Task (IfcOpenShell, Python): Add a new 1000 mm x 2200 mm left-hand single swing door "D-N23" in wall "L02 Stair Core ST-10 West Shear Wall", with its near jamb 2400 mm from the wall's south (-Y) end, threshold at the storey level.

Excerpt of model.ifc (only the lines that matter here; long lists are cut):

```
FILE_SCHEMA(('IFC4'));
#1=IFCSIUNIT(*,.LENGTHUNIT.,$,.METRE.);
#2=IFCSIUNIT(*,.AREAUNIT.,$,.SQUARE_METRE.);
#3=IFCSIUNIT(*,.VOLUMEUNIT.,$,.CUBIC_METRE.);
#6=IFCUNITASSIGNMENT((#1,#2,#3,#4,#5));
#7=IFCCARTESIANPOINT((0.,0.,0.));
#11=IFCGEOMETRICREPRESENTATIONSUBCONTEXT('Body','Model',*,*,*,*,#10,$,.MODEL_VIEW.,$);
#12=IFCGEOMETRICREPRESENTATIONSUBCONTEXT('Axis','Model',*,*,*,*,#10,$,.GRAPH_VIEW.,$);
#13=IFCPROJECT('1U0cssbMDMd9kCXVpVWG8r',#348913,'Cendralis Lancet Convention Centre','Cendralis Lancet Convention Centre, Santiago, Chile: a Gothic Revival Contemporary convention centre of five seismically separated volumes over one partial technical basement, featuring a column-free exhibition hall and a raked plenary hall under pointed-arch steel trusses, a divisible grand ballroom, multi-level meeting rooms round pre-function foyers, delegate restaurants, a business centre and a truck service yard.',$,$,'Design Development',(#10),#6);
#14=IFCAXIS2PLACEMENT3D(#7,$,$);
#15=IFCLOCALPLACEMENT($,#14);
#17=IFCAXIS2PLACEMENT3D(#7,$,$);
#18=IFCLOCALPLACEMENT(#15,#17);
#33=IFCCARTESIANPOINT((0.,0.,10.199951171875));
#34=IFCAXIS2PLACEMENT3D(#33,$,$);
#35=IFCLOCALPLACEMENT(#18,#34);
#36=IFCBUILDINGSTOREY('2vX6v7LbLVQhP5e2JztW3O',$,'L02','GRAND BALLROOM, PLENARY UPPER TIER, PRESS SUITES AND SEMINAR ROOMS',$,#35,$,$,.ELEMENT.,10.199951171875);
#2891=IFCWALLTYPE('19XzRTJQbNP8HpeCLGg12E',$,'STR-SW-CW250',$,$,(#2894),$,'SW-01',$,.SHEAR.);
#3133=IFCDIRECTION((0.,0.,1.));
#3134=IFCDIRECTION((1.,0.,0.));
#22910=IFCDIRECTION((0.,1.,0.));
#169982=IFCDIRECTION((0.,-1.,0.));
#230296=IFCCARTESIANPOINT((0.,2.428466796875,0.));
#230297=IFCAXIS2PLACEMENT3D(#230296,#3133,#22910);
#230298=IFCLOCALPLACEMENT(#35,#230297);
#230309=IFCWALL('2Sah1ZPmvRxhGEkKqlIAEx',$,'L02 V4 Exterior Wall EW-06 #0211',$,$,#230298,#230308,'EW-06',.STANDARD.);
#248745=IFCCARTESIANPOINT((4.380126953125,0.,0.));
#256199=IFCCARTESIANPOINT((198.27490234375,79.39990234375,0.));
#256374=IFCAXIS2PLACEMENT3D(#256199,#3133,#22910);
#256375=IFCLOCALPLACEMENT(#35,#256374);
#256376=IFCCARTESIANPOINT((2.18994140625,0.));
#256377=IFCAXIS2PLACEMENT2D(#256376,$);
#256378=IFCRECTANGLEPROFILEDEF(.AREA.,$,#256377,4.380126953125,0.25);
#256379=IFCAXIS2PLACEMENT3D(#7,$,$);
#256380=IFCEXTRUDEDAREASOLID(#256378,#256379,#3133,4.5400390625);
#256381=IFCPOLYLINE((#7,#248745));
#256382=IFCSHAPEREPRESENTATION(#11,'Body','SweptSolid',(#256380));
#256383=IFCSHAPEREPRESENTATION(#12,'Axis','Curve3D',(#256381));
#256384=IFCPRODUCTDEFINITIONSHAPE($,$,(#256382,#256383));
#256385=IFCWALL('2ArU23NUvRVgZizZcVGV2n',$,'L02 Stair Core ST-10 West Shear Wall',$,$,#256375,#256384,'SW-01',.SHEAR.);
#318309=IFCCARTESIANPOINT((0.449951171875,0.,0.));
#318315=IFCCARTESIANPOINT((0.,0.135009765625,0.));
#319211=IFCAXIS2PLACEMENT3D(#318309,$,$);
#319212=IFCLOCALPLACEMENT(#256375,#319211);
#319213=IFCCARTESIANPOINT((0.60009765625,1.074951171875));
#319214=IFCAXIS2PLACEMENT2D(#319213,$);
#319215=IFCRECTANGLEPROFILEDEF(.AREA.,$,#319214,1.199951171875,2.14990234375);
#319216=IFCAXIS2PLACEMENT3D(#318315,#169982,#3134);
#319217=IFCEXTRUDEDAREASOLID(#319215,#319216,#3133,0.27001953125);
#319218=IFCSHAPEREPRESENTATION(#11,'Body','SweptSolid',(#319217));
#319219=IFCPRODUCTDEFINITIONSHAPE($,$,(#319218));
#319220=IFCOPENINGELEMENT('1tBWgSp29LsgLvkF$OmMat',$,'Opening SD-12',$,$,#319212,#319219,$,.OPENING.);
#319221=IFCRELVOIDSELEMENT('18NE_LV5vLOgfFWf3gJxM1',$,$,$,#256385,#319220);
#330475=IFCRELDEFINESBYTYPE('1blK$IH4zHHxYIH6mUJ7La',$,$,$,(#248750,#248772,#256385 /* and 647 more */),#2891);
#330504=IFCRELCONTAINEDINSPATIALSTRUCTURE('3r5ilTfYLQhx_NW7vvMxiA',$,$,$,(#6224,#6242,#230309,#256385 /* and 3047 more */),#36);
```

```python
import numpy as np
import ifcopenshell
import ifcopenshell.api.feature
import ifcopenshell.api.geometry
import ifcopenshell.api.root
import ifcopenshell.api.spatial
import ifcopenshell.geom
import ifcopenshell.util.element
import ifcopenshell.util.placement
import ifcopenshell.util.representation
import ifcopenshell.util.shape
import ifcopenshell.util.unit

model = ifcopenshell.open("model.ifc")
unit_scale = ifcopenshell.util.unit.calculate_unit_scale(model)
settings = ifcopenshell.geom.settings()


def volume(element):
    """Net volume in cubic metres, openings subtracted."""
    shape = ifcopenshell.geom.create_shape(settings, element)
    return ifcopenshell.util.shape.get_volume(shape.geometry)


wall = model.by_guid("2ArU23NUvRVgZizZcVGV2n")
storey = ifcopenshell.util.element.get_container(wall, ifc_class="IfcBuildingStorey")
context = ifcopenshell.util.representation.get_context(model, "Model", "Body", "MODEL_VIEW")
before = volume(wall)

width, height, from_end, sill = 1, 2.2, 2.4, 0.0  # metres

# The wall runs along its own X axis, and the end named is its -X end.
wall_shape = ifcopenshell.geom.create_shape(settings, wall)
x, y, z = ifcopenshell.util.shape.get_vertices(wall_shape.geometry).T
start = x.min() + from_end
face, thickness = float(y.min()), float(y.max() - y.min())
wall_matrix = ifcopenshell.util.placement.get_local_placement(wall.ObjectPlacement)
level = ifcopenshell.util.placement.get_local_placement(storey.ObjectPlacement)[2, 3]


def in_wall(x, y):
    """Placement at x, y metres in the wall's axes, at sill height."""
    matrix = wall_matrix.copy()
    matrix[:, 3] = wall_matrix @ np.array([x / unit_scale, y / unit_scale, 0.0, 1.0])
    matrix[2, 3] = level + sill / unit_scale
    return matrix


# Opening: a box that overshoots both wall faces by 50 mm.
opening = ifcopenshell.api.root.create_entity(model, ifc_class="IfcOpeningElement", predefined_type="OPENING")
box = ifcopenshell.api.geometry.add_wall_representation(
    model, context=context, length=width, height=height, thickness=thickness + 0.1
)
ifcopenshell.api.geometry.assign_representation(model, product=opening, representation=box)
ifcopenshell.api.geometry.edit_object_placement(model, product=opening, matrix=in_wall(start, face - 0.05), is_si=False)
ifcopenshell.api.feature.add_feature(model, feature=opening, element=wall)

door = ifcopenshell.api.root.create_entity(model, ifc_class="IfcDoor", name="D-N23", predefined_type="DOOR")
door.OverallWidth, door.OverallHeight = width / unit_scale, height / unit_scale
door.OperationType = "SINGLE_SWING_LEFT"
body = ifcopenshell.api.geometry.add_door_representation(
    model,
    context=context,
    overall_width=door.OverallWidth,
    overall_height=door.OverallHeight,
    operation_type="SINGLE_SWING_LEFT",
    lining_properties={"LiningDepth": thickness / unit_scale, "ThresholdDepth": thickness / unit_scale},
)
ifcopenshell.api.geometry.assign_representation(model, product=door, representation=body)
ifcopenshell.api.spatial.assign_container(model, products=[door], relating_structure=storey)
ifcopenshell.api.feature.add_filling(model, opening=opening, element=door)

# The lining spans the wall, so the door starts at the wall face.
ifcopenshell.api.geometry.edit_object_placement(model, product=door, matrix=in_wall(start, face), is_si=False)

after = volume(wall)

print(f"wall volume {before:.3f} -> {after:.3f} m3")

model.write("model_updated.ifc")
```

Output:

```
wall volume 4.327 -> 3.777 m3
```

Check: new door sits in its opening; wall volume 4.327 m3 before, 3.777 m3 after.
